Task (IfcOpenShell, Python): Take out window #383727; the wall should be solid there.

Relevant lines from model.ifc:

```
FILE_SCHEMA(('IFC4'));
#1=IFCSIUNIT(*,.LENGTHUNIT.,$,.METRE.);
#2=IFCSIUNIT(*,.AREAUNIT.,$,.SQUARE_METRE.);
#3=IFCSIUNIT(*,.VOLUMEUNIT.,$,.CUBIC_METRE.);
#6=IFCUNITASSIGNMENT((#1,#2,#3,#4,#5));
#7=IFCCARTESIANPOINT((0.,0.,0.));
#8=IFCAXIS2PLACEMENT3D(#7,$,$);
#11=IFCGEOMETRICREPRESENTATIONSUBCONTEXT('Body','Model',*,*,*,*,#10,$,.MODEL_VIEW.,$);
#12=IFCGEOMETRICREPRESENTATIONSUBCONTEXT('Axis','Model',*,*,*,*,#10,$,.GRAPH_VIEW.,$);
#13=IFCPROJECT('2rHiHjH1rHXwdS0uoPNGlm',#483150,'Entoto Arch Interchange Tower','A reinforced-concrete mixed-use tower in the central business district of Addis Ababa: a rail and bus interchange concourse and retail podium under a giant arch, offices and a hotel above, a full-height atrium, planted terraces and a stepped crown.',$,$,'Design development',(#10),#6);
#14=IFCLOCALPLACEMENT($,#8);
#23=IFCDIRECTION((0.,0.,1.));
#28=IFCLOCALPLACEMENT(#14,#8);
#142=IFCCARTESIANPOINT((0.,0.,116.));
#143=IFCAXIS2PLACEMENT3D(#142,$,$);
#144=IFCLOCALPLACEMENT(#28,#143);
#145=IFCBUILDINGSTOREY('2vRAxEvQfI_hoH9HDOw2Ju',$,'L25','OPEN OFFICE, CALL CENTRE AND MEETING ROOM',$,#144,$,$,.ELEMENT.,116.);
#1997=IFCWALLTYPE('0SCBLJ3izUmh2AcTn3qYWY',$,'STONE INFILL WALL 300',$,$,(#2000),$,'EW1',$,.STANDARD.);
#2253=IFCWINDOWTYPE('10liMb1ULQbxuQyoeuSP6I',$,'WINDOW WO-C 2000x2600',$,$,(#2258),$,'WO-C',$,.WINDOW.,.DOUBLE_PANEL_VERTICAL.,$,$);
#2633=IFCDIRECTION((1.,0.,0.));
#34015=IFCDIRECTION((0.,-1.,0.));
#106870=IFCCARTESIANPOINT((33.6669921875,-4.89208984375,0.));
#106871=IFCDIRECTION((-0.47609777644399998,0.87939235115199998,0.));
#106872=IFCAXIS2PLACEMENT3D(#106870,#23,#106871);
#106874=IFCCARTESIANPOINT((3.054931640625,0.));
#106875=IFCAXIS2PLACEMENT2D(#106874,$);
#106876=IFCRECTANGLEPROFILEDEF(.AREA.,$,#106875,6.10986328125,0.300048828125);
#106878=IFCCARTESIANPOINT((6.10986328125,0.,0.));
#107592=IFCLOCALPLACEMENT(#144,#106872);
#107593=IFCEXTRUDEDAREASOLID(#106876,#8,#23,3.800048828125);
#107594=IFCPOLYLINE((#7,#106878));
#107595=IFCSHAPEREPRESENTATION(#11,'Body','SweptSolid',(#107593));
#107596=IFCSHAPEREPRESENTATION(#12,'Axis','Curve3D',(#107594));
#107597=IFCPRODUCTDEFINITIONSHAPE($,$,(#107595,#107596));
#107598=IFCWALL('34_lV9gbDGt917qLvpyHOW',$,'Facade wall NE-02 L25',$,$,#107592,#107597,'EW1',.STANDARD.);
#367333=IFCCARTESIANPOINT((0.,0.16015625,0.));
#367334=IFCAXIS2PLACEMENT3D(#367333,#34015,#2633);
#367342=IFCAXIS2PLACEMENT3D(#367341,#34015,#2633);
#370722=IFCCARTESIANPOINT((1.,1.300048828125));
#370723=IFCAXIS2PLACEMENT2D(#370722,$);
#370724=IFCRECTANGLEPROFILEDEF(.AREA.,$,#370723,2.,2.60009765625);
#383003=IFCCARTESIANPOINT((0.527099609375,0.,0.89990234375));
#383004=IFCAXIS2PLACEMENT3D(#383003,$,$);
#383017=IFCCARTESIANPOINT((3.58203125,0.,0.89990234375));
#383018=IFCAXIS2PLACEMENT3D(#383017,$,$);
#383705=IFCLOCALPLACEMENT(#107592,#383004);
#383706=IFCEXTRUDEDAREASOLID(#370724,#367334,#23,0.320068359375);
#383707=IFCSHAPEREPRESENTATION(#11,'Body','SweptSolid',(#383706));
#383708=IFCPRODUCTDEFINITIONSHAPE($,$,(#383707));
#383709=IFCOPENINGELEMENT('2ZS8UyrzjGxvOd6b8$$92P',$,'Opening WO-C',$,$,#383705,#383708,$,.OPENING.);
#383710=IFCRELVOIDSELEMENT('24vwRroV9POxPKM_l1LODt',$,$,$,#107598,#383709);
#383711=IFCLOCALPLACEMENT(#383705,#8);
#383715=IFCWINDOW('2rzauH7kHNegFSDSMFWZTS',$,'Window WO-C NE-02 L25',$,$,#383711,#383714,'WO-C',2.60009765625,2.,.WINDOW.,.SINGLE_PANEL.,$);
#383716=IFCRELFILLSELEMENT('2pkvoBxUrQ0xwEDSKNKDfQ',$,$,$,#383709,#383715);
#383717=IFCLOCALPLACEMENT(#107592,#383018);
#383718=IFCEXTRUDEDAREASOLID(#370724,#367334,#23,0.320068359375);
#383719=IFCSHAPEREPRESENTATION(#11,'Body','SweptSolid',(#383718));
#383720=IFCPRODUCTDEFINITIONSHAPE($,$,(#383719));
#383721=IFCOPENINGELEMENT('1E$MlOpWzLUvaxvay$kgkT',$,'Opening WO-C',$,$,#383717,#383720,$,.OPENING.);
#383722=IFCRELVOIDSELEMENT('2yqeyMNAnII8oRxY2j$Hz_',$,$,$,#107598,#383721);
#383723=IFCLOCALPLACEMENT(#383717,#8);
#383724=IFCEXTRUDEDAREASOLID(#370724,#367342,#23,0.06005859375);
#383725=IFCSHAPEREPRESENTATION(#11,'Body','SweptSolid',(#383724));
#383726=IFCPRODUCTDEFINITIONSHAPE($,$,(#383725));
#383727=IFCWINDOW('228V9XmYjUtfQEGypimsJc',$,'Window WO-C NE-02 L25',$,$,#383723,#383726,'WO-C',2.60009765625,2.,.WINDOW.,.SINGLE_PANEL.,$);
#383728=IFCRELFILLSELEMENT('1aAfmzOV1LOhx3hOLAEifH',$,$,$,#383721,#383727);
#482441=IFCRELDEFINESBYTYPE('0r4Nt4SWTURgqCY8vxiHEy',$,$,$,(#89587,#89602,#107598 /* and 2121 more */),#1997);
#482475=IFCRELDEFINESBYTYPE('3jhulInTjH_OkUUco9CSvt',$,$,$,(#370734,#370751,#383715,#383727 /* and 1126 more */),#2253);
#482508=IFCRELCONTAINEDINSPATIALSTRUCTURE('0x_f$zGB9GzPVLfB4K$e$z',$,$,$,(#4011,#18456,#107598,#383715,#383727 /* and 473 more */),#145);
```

```python
import ifcopenshell
import ifcopenshell.api.feature
import ifcopenshell.api.root
import ifcopenshell.geom
import ifcopenshell.util.shape

model = ifcopenshell.open("model.ifc")
settings = ifcopenshell.geom.settings()


def volume(element):
    """Net volume in cubic metres, openings subtracted."""
    shape = ifcopenshell.geom.create_shape(settings, element)
    return ifcopenshell.util.shape.get_volume(shape.geometry)


window = model.by_guid("228V9XmYjUtfQEGypimsJc")
opening = window.FillsVoids[0].RelatingOpeningElement
wall = opening.VoidsElements[0].RelatingBuildingElement
before = volume(wall)

ifcopenshell.api.root.remove_product(model, product=window)
ifcopenshell.api.feature.remove_feature(model, feature=opening)

after = volume(wall)

print(f"wall volume {before:.3f} -> {after:.3f} m3")

model.write("model_updated.ifc")
```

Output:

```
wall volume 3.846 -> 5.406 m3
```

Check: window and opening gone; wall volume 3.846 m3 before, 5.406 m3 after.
